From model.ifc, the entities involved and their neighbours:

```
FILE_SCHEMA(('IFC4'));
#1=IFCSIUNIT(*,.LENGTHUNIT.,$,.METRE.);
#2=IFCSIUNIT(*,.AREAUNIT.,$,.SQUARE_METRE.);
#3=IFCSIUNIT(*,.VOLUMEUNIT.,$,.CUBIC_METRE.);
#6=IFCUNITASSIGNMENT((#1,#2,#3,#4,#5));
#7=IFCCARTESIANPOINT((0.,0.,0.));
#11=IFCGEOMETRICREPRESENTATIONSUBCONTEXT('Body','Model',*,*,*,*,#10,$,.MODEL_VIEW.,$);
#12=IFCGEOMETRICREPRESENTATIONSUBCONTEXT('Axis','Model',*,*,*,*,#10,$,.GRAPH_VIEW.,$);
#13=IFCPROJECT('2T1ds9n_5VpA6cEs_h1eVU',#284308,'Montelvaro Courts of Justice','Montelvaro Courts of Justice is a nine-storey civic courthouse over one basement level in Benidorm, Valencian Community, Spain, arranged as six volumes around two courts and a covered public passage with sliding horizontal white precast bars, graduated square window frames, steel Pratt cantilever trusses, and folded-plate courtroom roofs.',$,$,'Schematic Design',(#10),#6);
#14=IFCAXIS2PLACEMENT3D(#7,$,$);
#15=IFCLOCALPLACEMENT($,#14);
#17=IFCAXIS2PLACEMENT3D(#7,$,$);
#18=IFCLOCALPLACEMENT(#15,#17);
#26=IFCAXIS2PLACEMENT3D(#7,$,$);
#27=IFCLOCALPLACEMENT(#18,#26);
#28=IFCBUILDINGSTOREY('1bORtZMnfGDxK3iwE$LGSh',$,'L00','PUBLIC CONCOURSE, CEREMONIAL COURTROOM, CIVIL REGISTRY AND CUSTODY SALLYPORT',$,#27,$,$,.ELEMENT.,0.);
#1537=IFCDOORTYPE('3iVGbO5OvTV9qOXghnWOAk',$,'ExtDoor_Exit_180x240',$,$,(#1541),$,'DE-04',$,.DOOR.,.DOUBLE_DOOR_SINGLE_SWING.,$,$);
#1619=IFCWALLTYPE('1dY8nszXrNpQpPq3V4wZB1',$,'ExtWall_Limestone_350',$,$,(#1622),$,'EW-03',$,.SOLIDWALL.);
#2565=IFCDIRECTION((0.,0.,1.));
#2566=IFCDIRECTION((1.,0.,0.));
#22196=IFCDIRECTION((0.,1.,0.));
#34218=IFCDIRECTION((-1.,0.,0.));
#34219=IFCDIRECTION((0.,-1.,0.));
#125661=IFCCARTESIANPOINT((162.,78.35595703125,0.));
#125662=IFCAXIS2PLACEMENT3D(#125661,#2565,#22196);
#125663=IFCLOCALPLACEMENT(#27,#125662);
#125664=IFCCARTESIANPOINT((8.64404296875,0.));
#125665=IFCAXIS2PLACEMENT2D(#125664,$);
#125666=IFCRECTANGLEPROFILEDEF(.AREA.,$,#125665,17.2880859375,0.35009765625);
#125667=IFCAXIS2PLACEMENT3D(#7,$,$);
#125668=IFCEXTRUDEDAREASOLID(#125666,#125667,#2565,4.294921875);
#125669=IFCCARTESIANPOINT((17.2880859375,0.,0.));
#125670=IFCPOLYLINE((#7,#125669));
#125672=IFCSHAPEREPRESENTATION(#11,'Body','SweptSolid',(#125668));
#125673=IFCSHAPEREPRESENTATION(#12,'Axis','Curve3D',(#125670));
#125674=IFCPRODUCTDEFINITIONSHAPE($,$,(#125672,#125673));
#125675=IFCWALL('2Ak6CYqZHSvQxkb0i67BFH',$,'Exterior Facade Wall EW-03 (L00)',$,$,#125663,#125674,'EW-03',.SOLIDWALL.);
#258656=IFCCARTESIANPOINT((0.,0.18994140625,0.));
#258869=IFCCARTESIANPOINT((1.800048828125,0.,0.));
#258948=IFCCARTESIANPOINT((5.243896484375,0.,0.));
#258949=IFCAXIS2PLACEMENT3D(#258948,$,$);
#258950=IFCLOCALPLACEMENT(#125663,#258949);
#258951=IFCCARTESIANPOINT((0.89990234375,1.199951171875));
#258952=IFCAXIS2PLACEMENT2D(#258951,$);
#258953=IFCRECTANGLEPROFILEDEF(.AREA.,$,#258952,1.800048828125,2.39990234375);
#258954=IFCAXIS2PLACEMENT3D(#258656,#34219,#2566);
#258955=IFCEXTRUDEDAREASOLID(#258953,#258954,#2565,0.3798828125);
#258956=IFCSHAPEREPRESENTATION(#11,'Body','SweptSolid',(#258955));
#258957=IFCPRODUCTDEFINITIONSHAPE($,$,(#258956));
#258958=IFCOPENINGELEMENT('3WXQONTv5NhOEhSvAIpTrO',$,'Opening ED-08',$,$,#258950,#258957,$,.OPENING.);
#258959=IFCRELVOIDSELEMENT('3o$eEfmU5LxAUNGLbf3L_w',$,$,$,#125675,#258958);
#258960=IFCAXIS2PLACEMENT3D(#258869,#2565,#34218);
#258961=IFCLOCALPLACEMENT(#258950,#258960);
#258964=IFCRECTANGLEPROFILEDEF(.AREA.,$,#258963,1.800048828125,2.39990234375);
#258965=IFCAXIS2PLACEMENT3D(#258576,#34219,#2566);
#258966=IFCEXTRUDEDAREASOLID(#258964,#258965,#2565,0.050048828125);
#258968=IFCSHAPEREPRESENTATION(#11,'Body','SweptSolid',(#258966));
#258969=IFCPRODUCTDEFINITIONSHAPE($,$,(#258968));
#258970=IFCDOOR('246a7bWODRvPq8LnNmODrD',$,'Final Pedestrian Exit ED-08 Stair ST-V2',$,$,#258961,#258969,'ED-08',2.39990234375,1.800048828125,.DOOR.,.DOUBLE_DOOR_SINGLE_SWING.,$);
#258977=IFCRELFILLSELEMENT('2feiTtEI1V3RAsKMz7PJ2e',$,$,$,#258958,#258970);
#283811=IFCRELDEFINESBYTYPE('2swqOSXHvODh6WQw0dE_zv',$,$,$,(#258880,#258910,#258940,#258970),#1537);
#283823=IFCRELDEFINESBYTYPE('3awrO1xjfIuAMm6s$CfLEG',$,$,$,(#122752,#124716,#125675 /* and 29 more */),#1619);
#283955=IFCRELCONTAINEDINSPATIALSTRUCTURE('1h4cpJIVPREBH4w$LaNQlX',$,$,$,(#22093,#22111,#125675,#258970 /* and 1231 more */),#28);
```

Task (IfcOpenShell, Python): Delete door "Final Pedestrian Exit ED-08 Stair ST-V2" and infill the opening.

```python
import ifcopenshell
import ifcopenshell.api.feature
import ifcopenshell.api.root
import ifcopenshell.geom
import ifcopenshell.util.shape

model = ifcopenshell.open("model.ifc")
settings = ifcopenshell.geom.settings()


def volume(element):
    """Net volume in cubic metres, openings subtracted."""
    shape = ifcopenshell.geom.create_shape(settings, element)
    return ifcopenshell.util.shape.get_volume(shape.geometry)


door = model.by_guid("246a7bWODRvPq8LnNmODrD")
opening = door.FillsVoids[0].RelatingOpeningElement
wall = opening.VoidsElements[0].RelatingBuildingElement
before = volume(wall)

ifcopenshell.api.root.remove_product(model, product=door)
ifcopenshell.api.feature.remove_feature(model, feature=opening)

after = volume(wall)

print(f"wall volume {before:.3f} -> {after:.3f} m3")

model.write("model_edited.ifc")
```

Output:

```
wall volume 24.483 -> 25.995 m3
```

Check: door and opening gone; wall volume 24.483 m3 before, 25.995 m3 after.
